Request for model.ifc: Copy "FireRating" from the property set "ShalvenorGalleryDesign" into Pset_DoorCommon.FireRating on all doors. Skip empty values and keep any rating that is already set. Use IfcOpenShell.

First a look at what the model holds.

```python
import ifcopenshell
import ifcopenshell.util.element

model = ifcopenshell.open("model.ifc")
print(model.schema)
doors = model.by_type("IfcDoor")
print(len(doors), "doors")
for e in doors[:8]:
    source = ifcopenshell.util.element.get_pset(e, "ShalvenorGalleryDesign", "FireRating")
    target = ifcopenshell.util.element.get_pset(e, "Pset_DoorCommon", "FireRating")
    print(e.id(), repr(source), repr(target), sep=" | ")
```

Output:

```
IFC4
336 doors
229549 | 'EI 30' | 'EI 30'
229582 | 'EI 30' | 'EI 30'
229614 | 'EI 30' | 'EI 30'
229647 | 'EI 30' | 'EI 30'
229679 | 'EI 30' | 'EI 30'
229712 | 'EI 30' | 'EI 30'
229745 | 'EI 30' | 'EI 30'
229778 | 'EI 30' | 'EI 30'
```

```python
import ifcopenshell
import ifcopenshell.api.pset
import ifcopenshell.util.element

model = ifcopenshell.open("model.ifc")

count = 0
for e in model.by_type("IfcDoor"):
    value = ifcopenshell.util.element.get_pset(e, "ShalvenorGalleryDesign", "FireRating")
    current = ifcopenshell.util.element.get_pset(e, "Pset_DoorCommon", "FireRating")
    if not value or not value.strip() or current:
        continue
    # add_pset returns the element's existing set when there is one.
    pset = ifcopenshell.api.pset.add_pset(model, product=e, name="Pset_DoorCommon")
    ifcopenshell.api.pset.edit_pset(model, pset=pset, properties={"FireRating": value})
    count += 1

print(count, "doors updated")

model.write("model-out.ifc")
```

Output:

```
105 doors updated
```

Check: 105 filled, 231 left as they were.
